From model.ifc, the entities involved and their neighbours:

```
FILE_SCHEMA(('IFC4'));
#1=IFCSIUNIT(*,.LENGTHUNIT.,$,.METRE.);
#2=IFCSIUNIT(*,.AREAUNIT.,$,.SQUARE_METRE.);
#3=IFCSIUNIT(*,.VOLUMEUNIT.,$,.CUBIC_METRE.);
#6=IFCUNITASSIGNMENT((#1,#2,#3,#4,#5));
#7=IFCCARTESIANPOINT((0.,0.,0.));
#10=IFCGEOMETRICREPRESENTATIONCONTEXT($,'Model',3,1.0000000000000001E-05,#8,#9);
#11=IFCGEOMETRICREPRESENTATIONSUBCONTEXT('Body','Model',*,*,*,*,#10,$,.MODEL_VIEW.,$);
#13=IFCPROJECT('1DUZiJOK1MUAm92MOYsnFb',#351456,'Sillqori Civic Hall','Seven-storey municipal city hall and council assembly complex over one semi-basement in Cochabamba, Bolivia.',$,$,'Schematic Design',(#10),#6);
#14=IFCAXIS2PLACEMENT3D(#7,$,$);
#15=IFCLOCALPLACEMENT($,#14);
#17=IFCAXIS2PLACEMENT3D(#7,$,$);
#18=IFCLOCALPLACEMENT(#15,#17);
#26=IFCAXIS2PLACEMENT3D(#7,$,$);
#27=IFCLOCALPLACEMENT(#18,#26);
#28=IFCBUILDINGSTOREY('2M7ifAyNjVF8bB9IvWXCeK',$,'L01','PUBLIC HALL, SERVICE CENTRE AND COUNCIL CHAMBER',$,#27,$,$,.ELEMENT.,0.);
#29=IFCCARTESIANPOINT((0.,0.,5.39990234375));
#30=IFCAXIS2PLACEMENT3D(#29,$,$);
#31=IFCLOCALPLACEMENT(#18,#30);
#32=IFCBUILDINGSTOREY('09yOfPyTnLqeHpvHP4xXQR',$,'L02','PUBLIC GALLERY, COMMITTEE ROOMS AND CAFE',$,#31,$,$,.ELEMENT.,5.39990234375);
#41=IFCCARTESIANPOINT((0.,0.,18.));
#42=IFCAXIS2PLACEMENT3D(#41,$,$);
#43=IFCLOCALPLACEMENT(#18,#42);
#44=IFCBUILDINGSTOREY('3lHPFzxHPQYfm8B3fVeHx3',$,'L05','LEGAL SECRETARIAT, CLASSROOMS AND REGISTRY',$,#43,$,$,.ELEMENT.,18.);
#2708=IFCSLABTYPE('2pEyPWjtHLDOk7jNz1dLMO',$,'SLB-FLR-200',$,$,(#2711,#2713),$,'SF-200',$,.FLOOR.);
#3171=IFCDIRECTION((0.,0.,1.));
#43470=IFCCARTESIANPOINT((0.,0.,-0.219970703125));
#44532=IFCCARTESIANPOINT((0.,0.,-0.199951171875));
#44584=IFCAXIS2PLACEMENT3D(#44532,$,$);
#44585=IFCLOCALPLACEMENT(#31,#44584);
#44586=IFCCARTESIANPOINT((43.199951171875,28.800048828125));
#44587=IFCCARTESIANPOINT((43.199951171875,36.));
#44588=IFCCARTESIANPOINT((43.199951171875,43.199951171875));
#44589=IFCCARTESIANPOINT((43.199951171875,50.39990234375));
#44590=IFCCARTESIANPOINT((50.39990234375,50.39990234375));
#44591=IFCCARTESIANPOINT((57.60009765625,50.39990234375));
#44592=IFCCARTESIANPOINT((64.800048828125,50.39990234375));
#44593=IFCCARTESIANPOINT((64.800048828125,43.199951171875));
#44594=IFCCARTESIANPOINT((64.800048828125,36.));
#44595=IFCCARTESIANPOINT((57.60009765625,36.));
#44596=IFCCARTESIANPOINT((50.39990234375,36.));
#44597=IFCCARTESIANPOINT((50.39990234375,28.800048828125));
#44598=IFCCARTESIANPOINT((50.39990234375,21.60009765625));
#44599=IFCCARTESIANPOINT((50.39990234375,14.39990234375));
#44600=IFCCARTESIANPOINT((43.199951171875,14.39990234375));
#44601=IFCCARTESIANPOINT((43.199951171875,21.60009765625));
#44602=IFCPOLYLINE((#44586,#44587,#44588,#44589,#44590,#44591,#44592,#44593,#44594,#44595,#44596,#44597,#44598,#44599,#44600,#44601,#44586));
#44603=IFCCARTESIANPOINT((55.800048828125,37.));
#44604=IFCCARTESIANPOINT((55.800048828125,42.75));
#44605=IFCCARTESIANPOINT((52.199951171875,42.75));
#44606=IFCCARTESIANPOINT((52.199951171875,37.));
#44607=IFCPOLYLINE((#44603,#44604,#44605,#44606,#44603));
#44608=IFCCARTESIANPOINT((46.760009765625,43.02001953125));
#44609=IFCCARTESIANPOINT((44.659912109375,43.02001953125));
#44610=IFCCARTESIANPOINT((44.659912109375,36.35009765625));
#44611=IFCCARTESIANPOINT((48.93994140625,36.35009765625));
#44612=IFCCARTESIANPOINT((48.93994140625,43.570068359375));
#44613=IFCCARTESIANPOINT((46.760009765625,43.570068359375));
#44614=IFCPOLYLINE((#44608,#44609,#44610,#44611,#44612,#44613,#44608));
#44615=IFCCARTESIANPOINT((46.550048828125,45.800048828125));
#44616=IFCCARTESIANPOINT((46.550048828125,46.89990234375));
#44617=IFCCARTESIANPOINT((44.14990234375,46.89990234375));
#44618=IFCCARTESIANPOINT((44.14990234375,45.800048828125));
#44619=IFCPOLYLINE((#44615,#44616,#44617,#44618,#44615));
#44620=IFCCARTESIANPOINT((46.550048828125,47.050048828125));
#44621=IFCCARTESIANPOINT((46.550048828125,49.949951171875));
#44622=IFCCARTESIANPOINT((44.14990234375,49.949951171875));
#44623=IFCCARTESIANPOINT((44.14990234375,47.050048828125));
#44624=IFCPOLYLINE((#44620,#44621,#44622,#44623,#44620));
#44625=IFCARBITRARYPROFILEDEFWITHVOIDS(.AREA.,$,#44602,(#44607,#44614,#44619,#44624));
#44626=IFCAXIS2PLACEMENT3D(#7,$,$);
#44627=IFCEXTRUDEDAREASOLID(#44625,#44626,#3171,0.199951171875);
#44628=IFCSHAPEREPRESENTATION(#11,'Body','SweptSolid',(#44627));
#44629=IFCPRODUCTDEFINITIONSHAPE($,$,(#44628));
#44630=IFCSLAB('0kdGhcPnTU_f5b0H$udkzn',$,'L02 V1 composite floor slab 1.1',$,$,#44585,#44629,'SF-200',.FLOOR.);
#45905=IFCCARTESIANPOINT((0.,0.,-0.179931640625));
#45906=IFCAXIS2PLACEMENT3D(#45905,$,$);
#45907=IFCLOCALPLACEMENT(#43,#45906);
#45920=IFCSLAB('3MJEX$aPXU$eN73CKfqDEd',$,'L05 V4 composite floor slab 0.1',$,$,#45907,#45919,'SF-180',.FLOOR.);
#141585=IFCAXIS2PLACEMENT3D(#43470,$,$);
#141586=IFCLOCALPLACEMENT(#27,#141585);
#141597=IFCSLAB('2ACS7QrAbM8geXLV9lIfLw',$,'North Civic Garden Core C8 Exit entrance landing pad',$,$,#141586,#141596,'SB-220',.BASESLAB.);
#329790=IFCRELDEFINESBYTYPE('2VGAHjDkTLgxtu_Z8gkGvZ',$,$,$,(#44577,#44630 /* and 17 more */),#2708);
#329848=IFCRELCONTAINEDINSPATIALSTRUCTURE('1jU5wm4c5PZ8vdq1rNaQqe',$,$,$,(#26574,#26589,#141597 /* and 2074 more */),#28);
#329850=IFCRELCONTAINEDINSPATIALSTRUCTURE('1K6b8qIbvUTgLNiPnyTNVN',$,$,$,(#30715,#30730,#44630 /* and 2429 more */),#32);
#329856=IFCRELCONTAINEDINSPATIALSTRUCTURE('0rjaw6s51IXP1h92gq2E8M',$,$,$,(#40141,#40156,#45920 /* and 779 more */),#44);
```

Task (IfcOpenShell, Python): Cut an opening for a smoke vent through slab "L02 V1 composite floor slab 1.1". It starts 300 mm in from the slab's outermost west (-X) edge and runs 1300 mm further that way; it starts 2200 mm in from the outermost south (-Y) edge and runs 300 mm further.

```python
import numpy as np
import ifcopenshell
import ifcopenshell.api.feature
import ifcopenshell.api.geometry
import ifcopenshell.api.root
import ifcopenshell.geom
import ifcopenshell.util.placement
import ifcopenshell.util.representation
import ifcopenshell.util.shape
import ifcopenshell.util.unit

model = ifcopenshell.open("model.ifc")
unit_scale = ifcopenshell.util.unit.calculate_unit_scale(model)
settings = ifcopenshell.geom.settings()


def volume(element):
    """Net volume in cubic metres, openings subtracted."""
    shape = ifcopenshell.geom.create_shape(settings, element)
    return ifcopenshell.util.shape.get_volume(shape.geometry)


slab = model.by_guid("0kdGhcPnTU_f5b0H$udkzn")
before = volume(slab)

# Extent in the slab's own axes, in metres. The edges named are its -X and -Y sides.
slab_shape = ifcopenshell.geom.create_shape(settings, slab)
vertices = ifcopenshell.util.shape.get_vertices(slab_shape.geometry)
x_min, y_min, bottom = vertices.min(axis=0)
top = vertices[:, 2].max()

opening = ifcopenshell.api.root.create_entity(model, ifc_class="IfcOpeningElement", name="Smoke vent opening", predefined_type="OPENING")
context = ifcopenshell.util.representation.get_context(model, "Model", "Body", "MODEL_VIEW")
width, depth = 1.3, 0.3
outline = [(0.0, 0.0), (width, 0.0), (width, depth), (0.0, depth), (0.0, 0.0)]
# Overshoot both faces by 50 mm so the cut is clean.
shape = ifcopenshell.api.geometry.add_slab_representation(
    model, context=context, depth=top - bottom + 0.1, polyline=outline
)
ifcopenshell.api.geometry.assign_representation(model, product=opening, representation=shape)

matrix = ifcopenshell.util.placement.get_local_placement(slab.ObjectPlacement)
matrix[:, 3] = matrix @ np.append(np.array([x_min + 0.3, y_min + 2.2, bottom - 0.05]) / unit_scale, 1.0)
ifcopenshell.api.geometry.edit_object_placement(model, product=opening, matrix=matrix, is_si=False)
ifcopenshell.api.feature.add_feature(model, feature=opening, element=slab)

after = volume(slab)

print(f"slab volume {before:.3f} -> {after:.3f} m3")

model.write("model_v2.ifc")
```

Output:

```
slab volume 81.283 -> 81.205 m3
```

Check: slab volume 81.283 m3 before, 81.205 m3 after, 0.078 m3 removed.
